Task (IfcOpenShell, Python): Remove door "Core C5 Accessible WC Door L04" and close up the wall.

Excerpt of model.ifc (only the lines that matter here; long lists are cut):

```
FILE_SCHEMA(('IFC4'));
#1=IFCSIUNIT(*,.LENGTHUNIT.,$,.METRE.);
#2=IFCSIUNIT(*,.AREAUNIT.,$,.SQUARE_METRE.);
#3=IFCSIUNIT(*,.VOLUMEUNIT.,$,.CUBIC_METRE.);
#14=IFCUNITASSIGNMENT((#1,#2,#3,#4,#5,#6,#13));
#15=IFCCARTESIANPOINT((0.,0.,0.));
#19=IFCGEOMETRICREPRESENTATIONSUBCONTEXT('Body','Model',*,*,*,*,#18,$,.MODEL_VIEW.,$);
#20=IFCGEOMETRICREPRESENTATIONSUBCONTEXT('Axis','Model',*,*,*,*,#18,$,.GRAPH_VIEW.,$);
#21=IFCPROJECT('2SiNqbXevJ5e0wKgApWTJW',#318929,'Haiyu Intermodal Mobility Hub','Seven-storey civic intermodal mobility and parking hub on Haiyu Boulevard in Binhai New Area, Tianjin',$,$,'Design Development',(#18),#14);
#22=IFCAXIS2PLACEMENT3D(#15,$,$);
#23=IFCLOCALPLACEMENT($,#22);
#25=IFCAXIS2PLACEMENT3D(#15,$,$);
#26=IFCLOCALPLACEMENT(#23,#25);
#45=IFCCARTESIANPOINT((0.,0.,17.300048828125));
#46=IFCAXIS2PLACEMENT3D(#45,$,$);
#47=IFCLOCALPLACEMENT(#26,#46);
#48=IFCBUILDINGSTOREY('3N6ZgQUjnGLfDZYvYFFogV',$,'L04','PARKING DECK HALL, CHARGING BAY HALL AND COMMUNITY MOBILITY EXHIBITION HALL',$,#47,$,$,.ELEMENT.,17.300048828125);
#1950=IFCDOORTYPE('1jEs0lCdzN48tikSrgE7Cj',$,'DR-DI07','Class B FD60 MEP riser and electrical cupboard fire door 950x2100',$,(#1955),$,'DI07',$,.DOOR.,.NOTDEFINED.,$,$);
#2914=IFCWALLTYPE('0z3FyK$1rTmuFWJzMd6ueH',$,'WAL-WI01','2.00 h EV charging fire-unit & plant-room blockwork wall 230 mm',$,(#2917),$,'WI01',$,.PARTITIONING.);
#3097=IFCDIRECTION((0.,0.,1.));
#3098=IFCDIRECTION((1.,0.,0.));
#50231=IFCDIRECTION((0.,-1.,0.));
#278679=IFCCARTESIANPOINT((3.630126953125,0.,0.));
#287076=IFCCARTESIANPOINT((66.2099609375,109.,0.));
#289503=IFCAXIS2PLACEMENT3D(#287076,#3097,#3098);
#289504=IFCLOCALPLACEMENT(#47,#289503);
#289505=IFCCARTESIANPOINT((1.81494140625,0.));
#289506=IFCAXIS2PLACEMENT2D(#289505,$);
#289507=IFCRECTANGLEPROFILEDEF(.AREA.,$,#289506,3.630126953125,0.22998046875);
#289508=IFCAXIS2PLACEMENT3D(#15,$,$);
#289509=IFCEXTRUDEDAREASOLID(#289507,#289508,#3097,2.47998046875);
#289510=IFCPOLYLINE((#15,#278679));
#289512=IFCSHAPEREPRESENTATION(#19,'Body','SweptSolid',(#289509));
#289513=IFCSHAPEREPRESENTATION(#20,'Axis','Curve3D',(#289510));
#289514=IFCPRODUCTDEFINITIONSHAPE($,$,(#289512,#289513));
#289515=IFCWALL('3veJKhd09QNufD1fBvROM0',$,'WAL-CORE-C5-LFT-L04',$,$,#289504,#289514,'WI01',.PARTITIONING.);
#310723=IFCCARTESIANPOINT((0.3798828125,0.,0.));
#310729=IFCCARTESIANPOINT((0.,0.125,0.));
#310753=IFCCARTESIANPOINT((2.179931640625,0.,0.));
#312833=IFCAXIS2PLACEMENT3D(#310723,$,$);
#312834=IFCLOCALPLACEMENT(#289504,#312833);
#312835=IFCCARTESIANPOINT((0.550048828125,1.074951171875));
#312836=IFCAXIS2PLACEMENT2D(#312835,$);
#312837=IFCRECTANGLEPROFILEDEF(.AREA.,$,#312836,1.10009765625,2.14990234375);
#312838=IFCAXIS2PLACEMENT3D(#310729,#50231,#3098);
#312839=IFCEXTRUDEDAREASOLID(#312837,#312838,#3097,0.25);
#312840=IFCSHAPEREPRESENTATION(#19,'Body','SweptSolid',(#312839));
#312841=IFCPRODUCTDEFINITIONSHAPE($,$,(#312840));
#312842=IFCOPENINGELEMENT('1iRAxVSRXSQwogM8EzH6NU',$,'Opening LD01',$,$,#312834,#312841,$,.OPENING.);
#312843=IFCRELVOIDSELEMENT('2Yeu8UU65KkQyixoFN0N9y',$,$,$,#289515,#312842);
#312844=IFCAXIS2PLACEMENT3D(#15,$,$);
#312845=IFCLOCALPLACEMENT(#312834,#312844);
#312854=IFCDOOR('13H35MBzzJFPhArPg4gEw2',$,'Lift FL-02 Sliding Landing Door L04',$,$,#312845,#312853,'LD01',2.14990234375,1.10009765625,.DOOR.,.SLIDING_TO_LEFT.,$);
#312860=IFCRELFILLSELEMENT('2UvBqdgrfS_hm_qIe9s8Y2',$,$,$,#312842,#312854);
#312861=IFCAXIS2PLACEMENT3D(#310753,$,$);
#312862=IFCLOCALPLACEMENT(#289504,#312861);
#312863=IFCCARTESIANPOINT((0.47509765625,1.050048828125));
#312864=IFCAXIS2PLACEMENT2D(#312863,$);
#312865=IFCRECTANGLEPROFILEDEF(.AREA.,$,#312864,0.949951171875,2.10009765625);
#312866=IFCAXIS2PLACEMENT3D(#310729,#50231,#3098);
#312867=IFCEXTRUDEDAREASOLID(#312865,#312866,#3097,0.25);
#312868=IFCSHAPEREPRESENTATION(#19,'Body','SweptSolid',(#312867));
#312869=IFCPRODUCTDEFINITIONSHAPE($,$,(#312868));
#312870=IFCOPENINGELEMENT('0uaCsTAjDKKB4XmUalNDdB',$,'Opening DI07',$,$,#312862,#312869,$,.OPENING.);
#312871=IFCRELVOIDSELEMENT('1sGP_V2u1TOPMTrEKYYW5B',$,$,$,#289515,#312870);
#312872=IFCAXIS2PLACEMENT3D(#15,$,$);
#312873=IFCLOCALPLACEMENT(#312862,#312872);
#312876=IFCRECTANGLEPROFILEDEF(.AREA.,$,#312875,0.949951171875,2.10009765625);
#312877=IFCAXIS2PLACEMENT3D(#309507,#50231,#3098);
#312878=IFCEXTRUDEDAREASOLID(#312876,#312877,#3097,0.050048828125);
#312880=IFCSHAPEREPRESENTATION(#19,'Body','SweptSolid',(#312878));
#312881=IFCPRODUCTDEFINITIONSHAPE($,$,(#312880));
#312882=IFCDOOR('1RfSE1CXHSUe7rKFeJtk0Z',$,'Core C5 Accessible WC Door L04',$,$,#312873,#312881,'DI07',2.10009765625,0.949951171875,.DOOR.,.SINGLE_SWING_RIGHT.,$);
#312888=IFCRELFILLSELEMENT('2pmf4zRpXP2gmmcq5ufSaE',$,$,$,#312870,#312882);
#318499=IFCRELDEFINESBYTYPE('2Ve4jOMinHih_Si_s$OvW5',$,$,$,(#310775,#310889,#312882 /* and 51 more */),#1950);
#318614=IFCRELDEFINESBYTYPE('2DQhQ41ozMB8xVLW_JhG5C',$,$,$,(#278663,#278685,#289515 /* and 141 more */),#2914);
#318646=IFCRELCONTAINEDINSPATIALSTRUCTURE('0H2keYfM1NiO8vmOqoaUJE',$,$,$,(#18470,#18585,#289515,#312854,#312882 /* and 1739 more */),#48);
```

```python
import ifcopenshell
import ifcopenshell.api.feature
import ifcopenshell.api.root
import ifcopenshell.geom
import ifcopenshell.util.shape

model = ifcopenshell.open("model.ifc")
settings = ifcopenshell.geom.settings()


def volume(element):
    """Net volume in cubic metres, openings subtracted."""
    shape = ifcopenshell.geom.create_shape(settings, element)
    return ifcopenshell.util.shape.get_volume(shape.geometry)


door = model.by_guid("1RfSE1CXHSUe7rKFeJtk0Z")
opening = door.FillsVoids[0].RelatingOpeningElement
wall = opening.VoidsElements[0].RelatingBuildingElement
before = volume(wall)

ifcopenshell.api.root.remove_product(model, product=door)
ifcopenshell.api.feature.remove_feature(model, feature=opening)

after = volume(wall)

print(f"wall volume {before:.3f} -> {after:.3f} m3")

model.write("model_edited.ifc")
```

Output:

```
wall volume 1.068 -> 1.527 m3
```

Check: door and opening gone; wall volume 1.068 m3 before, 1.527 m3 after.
